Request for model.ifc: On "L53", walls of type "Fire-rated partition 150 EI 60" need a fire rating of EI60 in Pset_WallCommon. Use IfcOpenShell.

First a look at what the model holds.

```python
import ifcopenshell
import ifcopenshell.util.element

model = ifcopenshell.open("model.ifc")
print(model.schema)
storey = next(s for s in model.by_type("IfcBuildingStorey") if s.Name == "L53")
walls = [e for e in ifcopenshell.util.element.get_decomposition(storey) if e.is_a("IfcWall")]
seen = {}
for e in walls:
    element_type = ifcopenshell.util.element.get_type(e)
    key = (element_type.Name if element_type != e and element_type else None, ifcopenshell.util.element.get_pset(e, "Pset_WallCommon", "FireRating"))
    seen[key] = seen.get(key, 0) + 1
for (name, value), count in sorted(seen.items(), key=str):
    print(count, "x", name, "|", value)
```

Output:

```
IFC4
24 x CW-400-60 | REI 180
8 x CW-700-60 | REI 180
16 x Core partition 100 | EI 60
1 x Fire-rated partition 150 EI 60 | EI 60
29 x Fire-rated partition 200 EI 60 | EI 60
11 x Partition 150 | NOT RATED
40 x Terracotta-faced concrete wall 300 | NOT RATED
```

```python
import ifcopenshell
import ifcopenshell.api.pset
import ifcopenshell.util.element

model = ifcopenshell.open("model.ifc")

storey = next(s for s in model.by_type("IfcBuildingStorey") if s.Name == "L53")
walls = [e for e in ifcopenshell.util.element.get_decomposition(storey) if e.is_a("IfcWall")]

count = 0
for e in walls:
    element_type = ifcopenshell.util.element.get_type(e)
    if element_type in (None, e) or element_type.Name != "Fire-rated partition 150 EI 60":
        continue
    found = ifcopenshell.util.element.get_pset(e, "Pset_WallCommon", should_inherit=False)
    if found:
        pset = model.by_id(found["id"])
        if len(ifcopenshell.util.element.get_elements_by_pset(pset)) > 1:
            pset = ifcopenshell.api.pset.unshare_pset(model, products=[e], pset=pset)[0]
    else:
        pset = ifcopenshell.api.pset.add_pset(model, product=e, name="Pset_WallCommon")
    ifcopenshell.api.pset.edit_pset(model, pset=pset, properties={"FireRating": "EI60"})
    count += 1

print(count, "walls updated")

model.write("model_v2.ifc")
```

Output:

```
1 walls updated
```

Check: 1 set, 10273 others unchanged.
